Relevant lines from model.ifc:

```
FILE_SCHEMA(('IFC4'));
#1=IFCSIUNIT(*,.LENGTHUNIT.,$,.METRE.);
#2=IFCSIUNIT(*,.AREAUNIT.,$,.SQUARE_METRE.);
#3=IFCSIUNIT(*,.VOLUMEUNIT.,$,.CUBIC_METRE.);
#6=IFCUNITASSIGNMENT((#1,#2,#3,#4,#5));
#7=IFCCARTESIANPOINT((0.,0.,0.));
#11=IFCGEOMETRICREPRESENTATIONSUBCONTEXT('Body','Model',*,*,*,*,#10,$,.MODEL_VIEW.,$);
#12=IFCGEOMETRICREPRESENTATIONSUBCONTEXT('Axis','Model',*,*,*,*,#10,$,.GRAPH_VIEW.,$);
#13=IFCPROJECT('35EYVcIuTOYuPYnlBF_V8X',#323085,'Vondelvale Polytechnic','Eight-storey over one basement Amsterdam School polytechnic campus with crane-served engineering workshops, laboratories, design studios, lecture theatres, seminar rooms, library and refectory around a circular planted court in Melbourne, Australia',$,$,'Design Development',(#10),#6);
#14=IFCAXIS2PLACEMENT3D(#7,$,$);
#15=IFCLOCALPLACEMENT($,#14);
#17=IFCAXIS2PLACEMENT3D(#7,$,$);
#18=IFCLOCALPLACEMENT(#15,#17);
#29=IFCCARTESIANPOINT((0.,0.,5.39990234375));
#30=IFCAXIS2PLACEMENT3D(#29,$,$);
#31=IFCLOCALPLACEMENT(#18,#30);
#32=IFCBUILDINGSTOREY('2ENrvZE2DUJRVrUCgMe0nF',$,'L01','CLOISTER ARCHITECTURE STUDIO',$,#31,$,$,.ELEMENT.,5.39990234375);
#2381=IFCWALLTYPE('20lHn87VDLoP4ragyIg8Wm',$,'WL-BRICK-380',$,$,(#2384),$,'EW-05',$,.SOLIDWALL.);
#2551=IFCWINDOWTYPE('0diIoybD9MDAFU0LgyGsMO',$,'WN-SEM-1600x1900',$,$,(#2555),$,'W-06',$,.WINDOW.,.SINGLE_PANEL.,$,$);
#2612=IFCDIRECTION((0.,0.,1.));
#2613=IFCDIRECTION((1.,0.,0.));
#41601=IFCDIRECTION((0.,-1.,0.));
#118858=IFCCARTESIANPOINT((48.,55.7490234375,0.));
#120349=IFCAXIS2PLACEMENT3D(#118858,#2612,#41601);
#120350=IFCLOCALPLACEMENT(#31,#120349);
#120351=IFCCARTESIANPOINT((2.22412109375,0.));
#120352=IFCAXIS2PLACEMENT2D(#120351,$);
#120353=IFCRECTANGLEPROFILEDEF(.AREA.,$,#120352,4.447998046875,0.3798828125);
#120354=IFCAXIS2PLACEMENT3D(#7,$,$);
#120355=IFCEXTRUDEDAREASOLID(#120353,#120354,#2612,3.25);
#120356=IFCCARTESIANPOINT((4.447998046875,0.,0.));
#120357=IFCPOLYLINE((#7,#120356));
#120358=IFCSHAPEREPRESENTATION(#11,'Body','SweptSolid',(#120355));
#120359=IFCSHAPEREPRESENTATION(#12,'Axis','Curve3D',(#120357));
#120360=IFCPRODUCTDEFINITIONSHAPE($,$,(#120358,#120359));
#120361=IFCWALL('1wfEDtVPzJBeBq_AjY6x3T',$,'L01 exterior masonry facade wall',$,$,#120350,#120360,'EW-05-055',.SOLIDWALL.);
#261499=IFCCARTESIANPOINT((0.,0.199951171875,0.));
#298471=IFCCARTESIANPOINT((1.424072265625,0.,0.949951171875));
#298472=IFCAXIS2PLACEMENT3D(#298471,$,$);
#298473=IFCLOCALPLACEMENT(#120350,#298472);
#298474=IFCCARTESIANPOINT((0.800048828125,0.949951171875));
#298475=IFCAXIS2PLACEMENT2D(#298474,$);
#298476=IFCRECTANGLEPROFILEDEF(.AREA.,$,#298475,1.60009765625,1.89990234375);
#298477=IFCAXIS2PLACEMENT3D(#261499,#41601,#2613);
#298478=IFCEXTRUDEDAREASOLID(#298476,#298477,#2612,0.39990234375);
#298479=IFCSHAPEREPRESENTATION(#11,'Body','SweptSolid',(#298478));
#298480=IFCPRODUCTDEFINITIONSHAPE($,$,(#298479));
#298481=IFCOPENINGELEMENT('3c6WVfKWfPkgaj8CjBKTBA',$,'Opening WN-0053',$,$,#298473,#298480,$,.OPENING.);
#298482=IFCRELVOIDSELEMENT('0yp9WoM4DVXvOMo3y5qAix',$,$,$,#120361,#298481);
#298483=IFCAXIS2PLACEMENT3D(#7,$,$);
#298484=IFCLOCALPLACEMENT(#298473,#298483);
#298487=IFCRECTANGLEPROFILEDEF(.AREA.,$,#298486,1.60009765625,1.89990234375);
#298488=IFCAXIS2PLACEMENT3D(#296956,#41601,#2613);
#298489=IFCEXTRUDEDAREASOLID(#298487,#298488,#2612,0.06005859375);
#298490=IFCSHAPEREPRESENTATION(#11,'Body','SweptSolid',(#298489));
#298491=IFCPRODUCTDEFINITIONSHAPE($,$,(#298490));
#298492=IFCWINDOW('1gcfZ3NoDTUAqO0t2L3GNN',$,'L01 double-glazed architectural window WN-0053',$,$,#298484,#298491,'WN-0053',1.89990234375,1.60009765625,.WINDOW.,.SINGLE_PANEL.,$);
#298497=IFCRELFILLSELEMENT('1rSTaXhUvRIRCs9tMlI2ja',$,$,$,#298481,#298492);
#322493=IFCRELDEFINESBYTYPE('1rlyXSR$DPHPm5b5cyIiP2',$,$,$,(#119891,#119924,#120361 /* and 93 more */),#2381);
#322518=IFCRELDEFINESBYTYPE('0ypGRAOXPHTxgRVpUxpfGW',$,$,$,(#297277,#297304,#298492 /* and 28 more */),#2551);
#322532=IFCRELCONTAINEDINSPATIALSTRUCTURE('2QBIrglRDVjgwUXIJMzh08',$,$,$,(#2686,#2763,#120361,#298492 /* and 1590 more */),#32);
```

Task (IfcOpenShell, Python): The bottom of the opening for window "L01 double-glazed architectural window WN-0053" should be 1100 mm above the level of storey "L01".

```python
import numpy as np
import ifcopenshell
import ifcopenshell.api.geometry
import ifcopenshell.geom
import ifcopenshell.util.element
import ifcopenshell.util.placement
import ifcopenshell.util.shape
import ifcopenshell.util.unit

model = ifcopenshell.open("model.ifc")
unit_scale = ifcopenshell.util.unit.calculate_unit_scale(model)

window = model.by_id(298492)
opening = window.FillsVoids[0].RelatingOpeningElement
storey = ifcopenshell.util.element.get_container(window, ifc_class="IfcBuildingStorey")
level = ifcopenshell.util.placement.get_local_placement(storey.ObjectPlacement)[2, 3]

# The opening's origin need not be at the sill, so measure its lowest point.
shape = ifcopenshell.geom.create_shape(ifcopenshell.geom.settings(), opening)
bottom = ifcopenshell.util.shape.get_shape_bottom_elevation(shape, shape.geometry) / unit_scale
dz = level + 1.1 / unit_scale - bottom

shift = np.array([0.0, 0.0, dz])
# The window is placed relative to its opening, so it follows when the opening moves.
matrix = ifcopenshell.util.placement.get_local_placement(opening.ObjectPlacement)
matrix[:3, 3] += shift
ifcopenshell.api.geometry.edit_object_placement(
    model, product=opening, matrix=matrix, is_si=False, should_transform_children=True
)

print(f"moved by {dz * unit_scale:+.3f} m")

model.write("model_rev.ifc")
```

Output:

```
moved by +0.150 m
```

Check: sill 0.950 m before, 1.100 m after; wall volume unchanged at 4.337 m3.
